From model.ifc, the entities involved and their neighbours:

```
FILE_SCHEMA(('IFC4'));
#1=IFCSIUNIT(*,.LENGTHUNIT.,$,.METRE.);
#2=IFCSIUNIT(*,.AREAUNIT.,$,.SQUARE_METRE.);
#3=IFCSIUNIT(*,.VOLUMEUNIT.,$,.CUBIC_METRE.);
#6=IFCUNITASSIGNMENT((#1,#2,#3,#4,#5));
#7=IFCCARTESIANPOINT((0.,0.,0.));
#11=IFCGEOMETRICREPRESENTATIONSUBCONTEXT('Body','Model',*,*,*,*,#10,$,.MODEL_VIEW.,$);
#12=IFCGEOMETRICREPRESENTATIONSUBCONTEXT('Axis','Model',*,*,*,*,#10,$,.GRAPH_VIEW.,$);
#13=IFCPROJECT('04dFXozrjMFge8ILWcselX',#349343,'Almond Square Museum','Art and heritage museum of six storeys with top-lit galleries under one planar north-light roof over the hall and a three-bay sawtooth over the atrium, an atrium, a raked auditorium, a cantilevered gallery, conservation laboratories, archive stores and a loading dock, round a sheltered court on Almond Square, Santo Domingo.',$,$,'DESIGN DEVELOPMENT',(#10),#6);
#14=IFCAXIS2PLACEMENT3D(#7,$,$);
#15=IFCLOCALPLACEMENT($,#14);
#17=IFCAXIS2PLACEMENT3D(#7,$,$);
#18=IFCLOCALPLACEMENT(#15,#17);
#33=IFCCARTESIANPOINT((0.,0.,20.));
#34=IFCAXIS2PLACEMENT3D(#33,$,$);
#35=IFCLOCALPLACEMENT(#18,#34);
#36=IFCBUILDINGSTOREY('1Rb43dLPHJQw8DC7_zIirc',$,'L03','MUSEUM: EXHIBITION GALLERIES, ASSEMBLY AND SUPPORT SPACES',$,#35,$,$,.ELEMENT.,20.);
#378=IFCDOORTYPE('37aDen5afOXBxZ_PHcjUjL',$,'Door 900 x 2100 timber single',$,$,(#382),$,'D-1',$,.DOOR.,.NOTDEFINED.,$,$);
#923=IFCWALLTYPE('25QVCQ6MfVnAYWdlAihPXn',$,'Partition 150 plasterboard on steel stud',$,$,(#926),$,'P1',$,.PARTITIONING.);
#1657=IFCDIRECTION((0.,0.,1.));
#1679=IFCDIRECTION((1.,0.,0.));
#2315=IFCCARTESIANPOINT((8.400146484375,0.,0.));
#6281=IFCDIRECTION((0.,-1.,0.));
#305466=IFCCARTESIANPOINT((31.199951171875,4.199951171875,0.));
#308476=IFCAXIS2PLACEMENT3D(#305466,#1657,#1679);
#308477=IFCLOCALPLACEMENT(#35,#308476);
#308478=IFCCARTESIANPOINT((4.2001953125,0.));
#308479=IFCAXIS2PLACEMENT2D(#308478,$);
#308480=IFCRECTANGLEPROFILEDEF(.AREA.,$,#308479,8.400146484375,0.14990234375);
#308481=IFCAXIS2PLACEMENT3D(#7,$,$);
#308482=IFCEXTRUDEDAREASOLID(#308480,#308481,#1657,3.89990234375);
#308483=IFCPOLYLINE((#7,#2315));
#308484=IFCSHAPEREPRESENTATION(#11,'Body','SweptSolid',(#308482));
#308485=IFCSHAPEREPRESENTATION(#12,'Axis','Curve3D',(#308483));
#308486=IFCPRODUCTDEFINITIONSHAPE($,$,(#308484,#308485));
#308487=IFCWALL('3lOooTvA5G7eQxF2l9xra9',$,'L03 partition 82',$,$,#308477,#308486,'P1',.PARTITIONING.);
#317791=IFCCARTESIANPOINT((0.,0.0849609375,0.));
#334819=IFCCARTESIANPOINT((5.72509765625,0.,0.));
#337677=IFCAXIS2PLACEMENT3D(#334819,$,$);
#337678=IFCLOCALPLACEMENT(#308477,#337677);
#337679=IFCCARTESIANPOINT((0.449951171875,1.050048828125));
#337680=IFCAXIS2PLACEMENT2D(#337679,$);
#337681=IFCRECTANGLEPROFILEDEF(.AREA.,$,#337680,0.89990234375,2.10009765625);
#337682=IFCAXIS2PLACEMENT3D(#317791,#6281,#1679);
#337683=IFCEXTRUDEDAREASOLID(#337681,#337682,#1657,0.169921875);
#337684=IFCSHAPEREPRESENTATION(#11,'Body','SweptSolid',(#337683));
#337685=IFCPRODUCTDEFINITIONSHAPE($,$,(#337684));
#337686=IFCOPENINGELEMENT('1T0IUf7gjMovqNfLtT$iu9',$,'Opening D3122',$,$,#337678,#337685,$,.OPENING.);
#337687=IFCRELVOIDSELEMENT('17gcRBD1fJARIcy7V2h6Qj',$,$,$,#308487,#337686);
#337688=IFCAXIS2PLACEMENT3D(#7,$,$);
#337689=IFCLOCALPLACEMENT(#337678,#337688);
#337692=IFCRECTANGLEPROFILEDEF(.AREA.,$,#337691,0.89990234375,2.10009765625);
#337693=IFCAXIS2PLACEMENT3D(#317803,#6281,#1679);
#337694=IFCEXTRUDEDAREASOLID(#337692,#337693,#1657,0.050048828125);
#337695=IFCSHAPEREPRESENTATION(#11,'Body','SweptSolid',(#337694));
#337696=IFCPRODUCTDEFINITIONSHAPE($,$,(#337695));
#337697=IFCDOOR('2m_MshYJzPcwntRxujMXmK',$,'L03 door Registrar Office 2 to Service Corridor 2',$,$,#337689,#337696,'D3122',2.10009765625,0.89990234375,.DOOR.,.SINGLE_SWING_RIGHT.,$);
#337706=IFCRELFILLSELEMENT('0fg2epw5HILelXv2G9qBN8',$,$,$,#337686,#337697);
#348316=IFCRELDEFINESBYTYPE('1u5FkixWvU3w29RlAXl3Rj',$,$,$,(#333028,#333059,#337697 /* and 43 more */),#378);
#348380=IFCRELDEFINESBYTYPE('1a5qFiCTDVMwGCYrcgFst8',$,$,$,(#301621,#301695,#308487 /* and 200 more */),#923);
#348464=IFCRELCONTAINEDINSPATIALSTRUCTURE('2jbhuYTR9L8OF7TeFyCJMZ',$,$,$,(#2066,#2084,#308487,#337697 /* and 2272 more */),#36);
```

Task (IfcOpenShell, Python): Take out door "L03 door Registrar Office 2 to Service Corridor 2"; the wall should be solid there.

```python
import ifcopenshell
import ifcopenshell.api.feature
import ifcopenshell.api.root
import ifcopenshell.geom
import ifcopenshell.util.shape

model = ifcopenshell.open("model.ifc")
settings = ifcopenshell.geom.settings()


def volume(element):
    """Net volume in cubic metres, openings subtracted."""
    shape = ifcopenshell.geom.create_shape(settings, element)
    return ifcopenshell.util.shape.get_volume(shape.geometry)


door = model.by_guid("2m_MshYJzPcwntRxujMXmK")
opening = door.FillsVoids[0].RelatingOpeningElement
wall = opening.VoidsElements[0].RelatingBuildingElement
before = volume(wall)

ifcopenshell.api.root.remove_product(model, product=door)
ifcopenshell.api.feature.remove_feature(model, feature=opening)

after = volume(wall)

print(f"wall volume {before:.3f} -> {after:.3f} m3")

model.write("model_edited.ifc")
```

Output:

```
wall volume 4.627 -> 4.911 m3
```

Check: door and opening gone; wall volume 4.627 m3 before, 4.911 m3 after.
